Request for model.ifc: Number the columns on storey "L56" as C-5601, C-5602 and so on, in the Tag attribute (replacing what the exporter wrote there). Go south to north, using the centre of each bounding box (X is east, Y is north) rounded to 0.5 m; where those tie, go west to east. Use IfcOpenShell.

First a look at what the model holds.

```python
import ifcopenshell
import ifcopenshell.util.element
import ifcopenshell.util.placement

model = ifcopenshell.open("model.ifc")
print(model.schema)
storey = next(s for s in model.by_type("IfcBuildingStorey") if s.Name == "L56")
columns = [e for e in ifcopenshell.util.element.get_decomposition(storey) if e.is_a("IfcColumn")]
for e in sorted(columns, key=lambda e: e.id()):
    origin = ifcopenshell.util.placement.get_local_placement(e.ObjectPlacement)[:3, 3]
    print(e.id(), e.Tag, e.Name, origin.round(2) + 0.0, sep=" | ")
```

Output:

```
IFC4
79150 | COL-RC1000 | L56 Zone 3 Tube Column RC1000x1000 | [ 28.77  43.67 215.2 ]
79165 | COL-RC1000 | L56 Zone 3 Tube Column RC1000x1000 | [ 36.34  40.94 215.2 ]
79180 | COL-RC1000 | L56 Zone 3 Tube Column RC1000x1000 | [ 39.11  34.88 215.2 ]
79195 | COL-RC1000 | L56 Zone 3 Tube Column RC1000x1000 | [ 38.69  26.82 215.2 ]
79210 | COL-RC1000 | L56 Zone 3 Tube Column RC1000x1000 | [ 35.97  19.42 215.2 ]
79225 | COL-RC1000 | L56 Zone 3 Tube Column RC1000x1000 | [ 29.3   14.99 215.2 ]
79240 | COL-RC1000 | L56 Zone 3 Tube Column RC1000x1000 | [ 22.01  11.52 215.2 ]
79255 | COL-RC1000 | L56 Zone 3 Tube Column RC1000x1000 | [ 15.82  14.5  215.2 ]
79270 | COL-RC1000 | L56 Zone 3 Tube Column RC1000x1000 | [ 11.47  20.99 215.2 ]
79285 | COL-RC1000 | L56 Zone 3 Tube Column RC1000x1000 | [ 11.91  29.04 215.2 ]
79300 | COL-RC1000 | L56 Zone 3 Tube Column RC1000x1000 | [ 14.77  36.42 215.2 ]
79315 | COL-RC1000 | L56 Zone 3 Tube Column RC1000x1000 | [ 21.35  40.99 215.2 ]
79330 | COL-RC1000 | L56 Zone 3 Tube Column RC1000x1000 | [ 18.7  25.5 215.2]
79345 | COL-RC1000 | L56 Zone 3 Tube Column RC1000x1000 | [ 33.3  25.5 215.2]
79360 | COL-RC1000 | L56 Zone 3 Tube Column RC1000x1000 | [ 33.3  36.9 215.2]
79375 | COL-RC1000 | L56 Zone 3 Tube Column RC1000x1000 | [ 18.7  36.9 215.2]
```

```python
import ifcopenshell
import ifcopenshell.geom
import ifcopenshell.util.element
import ifcopenshell.util.shape

model = ifcopenshell.open("model.ifc")
settings = ifcopenshell.geom.settings()
settings.set("use-world-coords", True)


def centre(element):
    shape = ifcopenshell.geom.create_shape(settings, element)
    return ifcopenshell.util.shape.get_bbox_centroid(shape.geometry)


storey = next(s for s in model.by_type("IfcBuildingStorey") if s.Name == "L56")
columns = [e for e in ifcopenshell.util.element.get_decomposition(storey) if e.is_a("IfcColumn")]

# Insertion points can sit at a corner or the storey origin, so sort by the geometry (in metres).
centres = {e: centre(e) for e in columns}
columns.sort(key=lambda e: (round(centres[e][1] / 0.5), centres[e][0]))

for i, e in enumerate(columns, start=1):
    number = f"C-56{i:02d}"
    e.Tag = number
    print(e.id(), number)

model.write("model_edited.ifc")
```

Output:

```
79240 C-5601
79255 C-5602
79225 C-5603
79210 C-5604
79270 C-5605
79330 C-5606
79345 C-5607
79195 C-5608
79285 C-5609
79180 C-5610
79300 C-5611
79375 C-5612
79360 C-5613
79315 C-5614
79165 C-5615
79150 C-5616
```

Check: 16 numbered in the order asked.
